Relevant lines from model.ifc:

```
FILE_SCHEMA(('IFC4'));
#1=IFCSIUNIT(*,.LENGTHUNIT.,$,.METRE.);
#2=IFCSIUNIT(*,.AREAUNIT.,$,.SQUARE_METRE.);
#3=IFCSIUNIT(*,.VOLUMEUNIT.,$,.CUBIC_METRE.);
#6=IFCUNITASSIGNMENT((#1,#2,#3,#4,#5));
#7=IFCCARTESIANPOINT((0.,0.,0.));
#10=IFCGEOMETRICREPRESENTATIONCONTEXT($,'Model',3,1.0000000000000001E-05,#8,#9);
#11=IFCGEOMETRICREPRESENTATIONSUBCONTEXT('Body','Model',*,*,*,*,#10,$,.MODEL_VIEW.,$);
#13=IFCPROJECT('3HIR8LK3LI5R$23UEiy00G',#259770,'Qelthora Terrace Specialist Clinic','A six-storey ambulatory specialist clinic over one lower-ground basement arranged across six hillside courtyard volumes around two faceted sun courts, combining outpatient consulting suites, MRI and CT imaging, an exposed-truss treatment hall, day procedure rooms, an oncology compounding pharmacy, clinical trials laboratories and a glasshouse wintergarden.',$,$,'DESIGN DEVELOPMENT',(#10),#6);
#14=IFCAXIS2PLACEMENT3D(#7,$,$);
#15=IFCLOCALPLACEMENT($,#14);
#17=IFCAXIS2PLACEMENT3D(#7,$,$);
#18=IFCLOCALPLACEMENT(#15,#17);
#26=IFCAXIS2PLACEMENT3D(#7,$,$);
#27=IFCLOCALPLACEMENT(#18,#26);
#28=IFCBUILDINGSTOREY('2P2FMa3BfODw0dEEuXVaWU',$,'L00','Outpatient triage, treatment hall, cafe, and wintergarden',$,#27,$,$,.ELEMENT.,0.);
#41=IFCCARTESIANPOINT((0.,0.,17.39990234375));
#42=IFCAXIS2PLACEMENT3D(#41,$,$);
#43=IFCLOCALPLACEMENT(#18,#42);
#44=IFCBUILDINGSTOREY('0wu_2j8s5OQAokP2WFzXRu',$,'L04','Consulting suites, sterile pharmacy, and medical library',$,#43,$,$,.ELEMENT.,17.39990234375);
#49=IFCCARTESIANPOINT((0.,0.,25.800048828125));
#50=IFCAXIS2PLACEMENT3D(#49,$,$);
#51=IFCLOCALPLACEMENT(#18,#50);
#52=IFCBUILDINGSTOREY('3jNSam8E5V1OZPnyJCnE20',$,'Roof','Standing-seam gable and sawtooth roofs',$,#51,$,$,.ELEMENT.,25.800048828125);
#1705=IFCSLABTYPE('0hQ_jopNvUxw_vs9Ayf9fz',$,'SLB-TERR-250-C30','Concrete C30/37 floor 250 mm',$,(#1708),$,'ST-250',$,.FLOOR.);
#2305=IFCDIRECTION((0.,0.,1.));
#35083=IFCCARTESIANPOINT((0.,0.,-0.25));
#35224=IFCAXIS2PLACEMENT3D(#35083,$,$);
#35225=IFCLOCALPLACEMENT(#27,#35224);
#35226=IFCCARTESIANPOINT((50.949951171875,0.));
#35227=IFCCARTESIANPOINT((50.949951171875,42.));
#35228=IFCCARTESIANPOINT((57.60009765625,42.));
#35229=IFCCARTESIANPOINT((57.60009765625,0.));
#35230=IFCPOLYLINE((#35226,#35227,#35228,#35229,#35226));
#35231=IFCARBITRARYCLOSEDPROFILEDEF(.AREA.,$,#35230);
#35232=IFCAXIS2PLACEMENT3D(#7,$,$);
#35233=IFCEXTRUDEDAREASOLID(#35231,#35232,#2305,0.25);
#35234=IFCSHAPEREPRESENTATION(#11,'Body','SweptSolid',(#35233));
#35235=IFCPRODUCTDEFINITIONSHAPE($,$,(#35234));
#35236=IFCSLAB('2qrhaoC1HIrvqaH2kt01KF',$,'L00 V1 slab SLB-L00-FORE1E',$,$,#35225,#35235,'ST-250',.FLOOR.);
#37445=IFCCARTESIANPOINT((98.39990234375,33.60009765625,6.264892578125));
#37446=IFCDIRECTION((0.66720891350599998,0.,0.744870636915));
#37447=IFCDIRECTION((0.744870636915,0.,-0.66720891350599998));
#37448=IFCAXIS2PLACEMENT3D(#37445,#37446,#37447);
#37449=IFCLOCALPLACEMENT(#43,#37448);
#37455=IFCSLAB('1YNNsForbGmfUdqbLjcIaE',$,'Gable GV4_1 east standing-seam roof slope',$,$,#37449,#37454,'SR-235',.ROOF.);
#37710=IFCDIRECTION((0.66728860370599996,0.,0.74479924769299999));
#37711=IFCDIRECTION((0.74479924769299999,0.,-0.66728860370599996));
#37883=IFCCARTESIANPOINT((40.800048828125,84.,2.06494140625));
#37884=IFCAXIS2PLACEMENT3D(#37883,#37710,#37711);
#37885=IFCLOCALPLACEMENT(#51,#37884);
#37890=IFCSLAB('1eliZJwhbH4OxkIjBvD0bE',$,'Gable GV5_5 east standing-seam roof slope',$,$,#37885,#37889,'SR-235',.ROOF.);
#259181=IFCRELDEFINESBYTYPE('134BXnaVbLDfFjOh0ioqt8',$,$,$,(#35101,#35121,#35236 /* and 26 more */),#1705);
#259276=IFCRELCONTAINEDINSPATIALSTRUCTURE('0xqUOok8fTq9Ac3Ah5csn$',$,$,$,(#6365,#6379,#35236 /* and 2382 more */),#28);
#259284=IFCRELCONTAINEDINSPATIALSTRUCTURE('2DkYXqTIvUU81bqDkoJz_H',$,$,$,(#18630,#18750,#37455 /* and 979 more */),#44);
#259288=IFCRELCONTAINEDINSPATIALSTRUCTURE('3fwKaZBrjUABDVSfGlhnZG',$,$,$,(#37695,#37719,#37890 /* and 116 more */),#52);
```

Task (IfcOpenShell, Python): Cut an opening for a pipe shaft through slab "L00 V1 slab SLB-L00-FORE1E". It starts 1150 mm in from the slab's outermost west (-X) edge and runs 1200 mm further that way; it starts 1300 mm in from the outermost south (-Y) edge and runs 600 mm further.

```python
import numpy as np
import ifcopenshell
import ifcopenshell.api.feature
import ifcopenshell.api.geometry
import ifcopenshell.api.root
import ifcopenshell.geom
import ifcopenshell.util.placement
import ifcopenshell.util.representation
import ifcopenshell.util.shape
import ifcopenshell.util.unit

model = ifcopenshell.open("model.ifc")
unit_scale = ifcopenshell.util.unit.calculate_unit_scale(model)
settings = ifcopenshell.geom.settings()


def volume(element):
    """Net volume in cubic metres, openings subtracted."""
    shape = ifcopenshell.geom.create_shape(settings, element)
    return ifcopenshell.util.shape.get_volume(shape.geometry)


slab = model.by_id(35236)
before = volume(slab)

# Extent in the slab's own axes, in metres. The edges named are its -X and -Y sides.
slab_shape = ifcopenshell.geom.create_shape(settings, slab)
vertices = ifcopenshell.util.shape.get_vertices(slab_shape.geometry)
x_min, y_min, bottom = vertices.min(axis=0)
top = vertices[:, 2].max()

opening = ifcopenshell.api.root.create_entity(model, ifc_class="IfcOpeningElement", name="Pipe shaft opening", predefined_type="OPENING")
context = ifcopenshell.util.representation.get_context(model, "Model", "Body", "MODEL_VIEW")
width, depth = 1.2, 0.6
outline = [(0.0, 0.0), (width, 0.0), (width, depth), (0.0, depth), (0.0, 0.0)]
# Overshoot both faces by 50 mm so the cut is clean.
shape = ifcopenshell.api.geometry.add_slab_representation(
    model, context=context, depth=top - bottom + 0.1, polyline=outline
)
ifcopenshell.api.geometry.assign_representation(model, product=opening, representation=shape)

matrix = ifcopenshell.util.placement.get_local_placement(slab.ObjectPlacement)
matrix[:, 3] = matrix @ np.append(np.array([x_min + 1.15, y_min + 1.3, bottom - 0.05]) / unit_scale, 1.0)
ifcopenshell.api.geometry.edit_object_placement(model, product=opening, matrix=matrix, is_si=False)
ifcopenshell.api.feature.add_feature(model, feature=opening, element=slab)

after = volume(slab)

print(f"slab volume {before:.3f} -> {after:.3f} m3")

model.write("model_v2.ifc")
```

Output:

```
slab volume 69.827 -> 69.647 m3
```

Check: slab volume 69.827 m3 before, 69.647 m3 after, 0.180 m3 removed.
